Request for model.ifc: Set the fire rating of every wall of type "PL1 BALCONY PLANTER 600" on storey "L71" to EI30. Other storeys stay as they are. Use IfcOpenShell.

First a look at what the model holds.

```python
import ifcopenshell
import ifcopenshell.util.element

model = ifcopenshell.open("model.ifc")
print(model.schema)
storey = next(s for s in model.by_type("IfcBuildingStorey") if s.Name == "L71")
walls = [e for e in ifcopenshell.util.element.get_decomposition(storey) if e.is_a("IfcWall")]
seen = {}
for e in walls:
    element_type = ifcopenshell.util.element.get_type(e)
    key = (element_type.Name if element_type != e and element_type else None, ifcopenshell.util.element.get_pset(e, "Pset_WallCommon", "FireRating"))
    seen[key] = seen.get(key, 0) + 1
for (name, value), count in sorted(seen.items(), key=str):
    print(count, "x", name, "|", value)
```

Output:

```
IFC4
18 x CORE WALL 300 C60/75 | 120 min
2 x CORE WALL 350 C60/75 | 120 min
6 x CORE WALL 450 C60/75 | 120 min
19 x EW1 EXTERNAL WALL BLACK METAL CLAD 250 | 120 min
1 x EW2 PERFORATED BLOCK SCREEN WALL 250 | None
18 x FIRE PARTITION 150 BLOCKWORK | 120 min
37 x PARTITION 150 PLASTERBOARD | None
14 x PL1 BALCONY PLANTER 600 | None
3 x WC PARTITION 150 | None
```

```python
import ifcopenshell
import ifcopenshell.api.pset
import ifcopenshell.util.element

model = ifcopenshell.open("model.ifc")

storey = next(s for s in model.by_type("IfcBuildingStorey") if s.Name == "L71")
walls = [e for e in ifcopenshell.util.element.get_decomposition(storey) if e.is_a("IfcWall")]

count = 0
for e in walls:
    element_type = ifcopenshell.util.element.get_type(e)
    if element_type in (None, e) or element_type.Name != "PL1 BALCONY PLANTER 600":
        continue
    found = ifcopenshell.util.element.get_pset(e, "Pset_WallCommon", should_inherit=False)
    if found:
        pset = model.by_id(found["id"])
        if len(ifcopenshell.util.element.get_elements_by_pset(pset)) > 1:
            pset = ifcopenshell.api.pset.unshare_pset(model, products=[e], pset=pset)[0]
    else:
        pset = ifcopenshell.api.pset.add_pset(model, product=e, name="Pset_WallCommon")
    ifcopenshell.api.pset.edit_pset(model, pset=pset, properties={"FireRating": "EI30"})
    count += 1

print(count, "walls updated")

model.write("model_rev.ifc")
```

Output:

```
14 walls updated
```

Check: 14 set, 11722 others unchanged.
